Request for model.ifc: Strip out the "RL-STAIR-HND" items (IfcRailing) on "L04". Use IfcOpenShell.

First a look at what the model holds.

```python
import ifcopenshell
import ifcopenshell.util.element

model = ifcopenshell.open("model.ifc")
print(model.schema)
storey = next(s for s in model.by_type("IfcBuildingStorey") if s.Name == "L04")
railings = [e for e in ifcopenshell.util.element.get_decomposition(storey) if e.is_a("IfcRailing")]
seen = {}
for e in railings:
    element_type = ifcopenshell.util.element.get_type(e)
    name = element_type.Name if element_type not in (None, e) else None
    seen[name] = seen.get(name, 0) + 1
for name, count in sorted(seen.items(), key=str):
    print(count, "x", name)
```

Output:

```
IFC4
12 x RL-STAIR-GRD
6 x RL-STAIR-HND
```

```python
import ifcopenshell
import ifcopenshell.api.root
import ifcopenshell.util.element

model = ifcopenshell.open("model.ifc")

storey = next(s for s in model.by_type("IfcBuildingStorey") if s.Name == "L04")
railings = [e for e in ifcopenshell.util.element.get_decomposition(storey) if e.is_a("IfcRailing")]
targets = [e for e in railings if (t := ifcopenshell.util.element.get_type(e)) not in (None, e) and t.Name == "RL-STAIR-HND"]

for e in targets:
    ifcopenshell.api.root.remove_product(model, product=e)
print(len(targets), "removed")

model.write("model_edited.ifc")
```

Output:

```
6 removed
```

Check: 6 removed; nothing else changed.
